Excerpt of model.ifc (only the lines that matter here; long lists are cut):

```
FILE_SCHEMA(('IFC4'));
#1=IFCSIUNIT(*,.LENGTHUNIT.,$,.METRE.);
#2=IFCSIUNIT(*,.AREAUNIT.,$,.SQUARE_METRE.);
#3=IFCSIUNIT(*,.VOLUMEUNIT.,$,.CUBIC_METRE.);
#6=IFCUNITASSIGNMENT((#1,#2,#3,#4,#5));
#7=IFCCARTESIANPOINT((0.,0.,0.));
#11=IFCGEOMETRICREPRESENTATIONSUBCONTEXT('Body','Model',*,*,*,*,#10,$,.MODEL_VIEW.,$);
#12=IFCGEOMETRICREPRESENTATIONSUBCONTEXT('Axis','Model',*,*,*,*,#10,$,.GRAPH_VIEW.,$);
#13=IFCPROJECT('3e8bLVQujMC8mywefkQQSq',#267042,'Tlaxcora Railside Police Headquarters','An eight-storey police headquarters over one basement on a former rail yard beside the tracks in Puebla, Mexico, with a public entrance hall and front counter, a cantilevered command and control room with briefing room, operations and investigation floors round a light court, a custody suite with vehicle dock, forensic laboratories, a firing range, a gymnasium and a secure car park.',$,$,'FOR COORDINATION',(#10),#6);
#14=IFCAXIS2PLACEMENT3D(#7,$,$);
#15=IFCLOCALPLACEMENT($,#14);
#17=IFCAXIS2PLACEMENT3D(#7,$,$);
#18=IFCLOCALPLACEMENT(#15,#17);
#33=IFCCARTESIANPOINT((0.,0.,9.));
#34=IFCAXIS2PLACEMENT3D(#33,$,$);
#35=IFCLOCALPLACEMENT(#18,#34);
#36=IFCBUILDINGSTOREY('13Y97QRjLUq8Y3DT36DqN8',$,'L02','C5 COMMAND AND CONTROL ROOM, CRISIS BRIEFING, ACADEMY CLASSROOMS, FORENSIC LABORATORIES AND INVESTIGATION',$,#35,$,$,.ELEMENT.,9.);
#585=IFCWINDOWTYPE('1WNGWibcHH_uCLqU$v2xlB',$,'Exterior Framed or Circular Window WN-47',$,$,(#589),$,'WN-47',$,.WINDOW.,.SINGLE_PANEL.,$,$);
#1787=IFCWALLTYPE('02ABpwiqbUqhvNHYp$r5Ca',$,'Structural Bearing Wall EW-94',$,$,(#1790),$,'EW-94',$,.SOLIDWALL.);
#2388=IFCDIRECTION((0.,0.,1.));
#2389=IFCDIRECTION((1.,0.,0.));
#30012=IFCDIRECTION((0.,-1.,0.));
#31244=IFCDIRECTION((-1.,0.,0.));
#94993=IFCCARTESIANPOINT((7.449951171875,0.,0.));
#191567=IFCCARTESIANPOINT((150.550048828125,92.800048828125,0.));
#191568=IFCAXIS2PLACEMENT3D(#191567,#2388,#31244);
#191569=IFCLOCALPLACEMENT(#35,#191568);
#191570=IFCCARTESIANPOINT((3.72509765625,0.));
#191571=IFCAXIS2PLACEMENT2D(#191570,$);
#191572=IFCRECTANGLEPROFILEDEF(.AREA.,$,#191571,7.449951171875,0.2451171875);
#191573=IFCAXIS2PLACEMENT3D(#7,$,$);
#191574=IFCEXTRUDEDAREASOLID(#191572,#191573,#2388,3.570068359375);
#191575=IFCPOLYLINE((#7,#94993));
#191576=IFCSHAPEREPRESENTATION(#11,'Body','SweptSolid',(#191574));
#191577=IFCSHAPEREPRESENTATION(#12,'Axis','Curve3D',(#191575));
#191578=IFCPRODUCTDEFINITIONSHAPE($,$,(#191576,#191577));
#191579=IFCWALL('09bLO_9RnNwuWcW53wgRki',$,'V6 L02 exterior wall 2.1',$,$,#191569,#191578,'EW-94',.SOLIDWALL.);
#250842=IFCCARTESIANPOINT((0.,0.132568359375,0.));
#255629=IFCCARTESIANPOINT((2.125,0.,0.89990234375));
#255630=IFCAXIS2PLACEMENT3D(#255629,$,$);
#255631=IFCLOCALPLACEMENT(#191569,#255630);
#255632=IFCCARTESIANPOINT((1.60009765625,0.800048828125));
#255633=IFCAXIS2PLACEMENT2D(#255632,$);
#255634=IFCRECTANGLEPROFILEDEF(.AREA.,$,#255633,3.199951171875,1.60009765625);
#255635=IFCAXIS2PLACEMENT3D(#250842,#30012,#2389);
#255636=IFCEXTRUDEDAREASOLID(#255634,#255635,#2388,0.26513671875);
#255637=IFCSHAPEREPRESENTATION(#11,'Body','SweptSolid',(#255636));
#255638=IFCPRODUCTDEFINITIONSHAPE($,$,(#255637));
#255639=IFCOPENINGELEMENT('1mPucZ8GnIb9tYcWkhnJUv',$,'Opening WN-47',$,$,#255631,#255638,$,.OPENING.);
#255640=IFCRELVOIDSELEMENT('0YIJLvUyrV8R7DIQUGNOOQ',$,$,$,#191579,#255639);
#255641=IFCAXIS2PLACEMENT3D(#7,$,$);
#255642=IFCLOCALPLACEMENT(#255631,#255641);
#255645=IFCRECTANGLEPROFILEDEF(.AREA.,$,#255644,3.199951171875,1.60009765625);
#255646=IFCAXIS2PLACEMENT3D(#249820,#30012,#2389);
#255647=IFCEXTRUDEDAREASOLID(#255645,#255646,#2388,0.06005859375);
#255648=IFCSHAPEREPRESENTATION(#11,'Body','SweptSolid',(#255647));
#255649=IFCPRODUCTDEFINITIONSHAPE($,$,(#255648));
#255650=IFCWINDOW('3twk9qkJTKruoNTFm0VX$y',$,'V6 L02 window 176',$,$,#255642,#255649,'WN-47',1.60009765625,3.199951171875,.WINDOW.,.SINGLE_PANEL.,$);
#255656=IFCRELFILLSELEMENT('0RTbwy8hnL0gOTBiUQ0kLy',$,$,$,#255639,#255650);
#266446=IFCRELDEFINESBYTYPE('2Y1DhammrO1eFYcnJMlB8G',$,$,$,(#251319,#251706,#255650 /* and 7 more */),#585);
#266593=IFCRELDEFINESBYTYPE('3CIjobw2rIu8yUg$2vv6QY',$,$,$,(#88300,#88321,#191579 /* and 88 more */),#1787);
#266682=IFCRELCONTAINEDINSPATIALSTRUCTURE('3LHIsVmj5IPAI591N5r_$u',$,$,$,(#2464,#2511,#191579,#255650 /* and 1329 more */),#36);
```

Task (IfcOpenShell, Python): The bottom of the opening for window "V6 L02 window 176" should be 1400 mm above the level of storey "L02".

```python
import numpy as np
import ifcopenshell
import ifcopenshell.api.geometry
import ifcopenshell.geom
import ifcopenshell.util.element
import ifcopenshell.util.placement
import ifcopenshell.util.shape
import ifcopenshell.util.unit

model = ifcopenshell.open("model.ifc")
unit_scale = ifcopenshell.util.unit.calculate_unit_scale(model)

window = model.by_id(255650)
opening = window.FillsVoids[0].RelatingOpeningElement
storey = ifcopenshell.util.element.get_container(window, ifc_class="IfcBuildingStorey")
level = ifcopenshell.util.placement.get_local_placement(storey.ObjectPlacement)[2, 3]

# The opening's origin need not be at the sill, so measure its lowest point.
shape = ifcopenshell.geom.create_shape(ifcopenshell.geom.settings(), opening)
bottom = ifcopenshell.util.shape.get_shape_bottom_elevation(shape, shape.geometry) / unit_scale
dz = level + 1.4 - bottom

shift = np.array([0.0, 0.0, dz])
# The window is placed relative to its opening, so it follows when the opening moves.
matrix = ifcopenshell.util.placement.get_local_placement(opening.ObjectPlacement)
matrix[:3, 3] += shift
ifcopenshell.api.geometry.edit_object_placement(
    model, product=opening, matrix=matrix, is_si=False, should_transform_children=True
)

print(f"moved by {dz * unit_scale:+.3f} m")

model.write("model_updated.ifc")
```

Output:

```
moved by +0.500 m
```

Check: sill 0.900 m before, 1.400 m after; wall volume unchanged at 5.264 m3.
